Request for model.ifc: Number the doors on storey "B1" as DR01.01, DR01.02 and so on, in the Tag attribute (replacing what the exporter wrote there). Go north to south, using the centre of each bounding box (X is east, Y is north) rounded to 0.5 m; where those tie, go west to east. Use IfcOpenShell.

First a look at what the model holds.

```python
import ifcopenshell
import ifcopenshell.util.element
import ifcopenshell.util.placement

model = ifcopenshell.open("model.ifc")
print(model.schema)
storey = next(s for s in model.by_type("IfcBuildingStorey") if s.Name == "B1")
doors = [e for e in ifcopenshell.util.element.get_decomposition(storey) if e.is_a("IfcDoor")]
for e in sorted(doors, key=lambda e: e.id()):
    origin = ifcopenshell.util.placement.get_local_placement(e.ObjectPlacement)[:3, 3]
    print(e.id(), e.Tag, e.Name, origin.round(2) + 0.0, sep=" | ")
```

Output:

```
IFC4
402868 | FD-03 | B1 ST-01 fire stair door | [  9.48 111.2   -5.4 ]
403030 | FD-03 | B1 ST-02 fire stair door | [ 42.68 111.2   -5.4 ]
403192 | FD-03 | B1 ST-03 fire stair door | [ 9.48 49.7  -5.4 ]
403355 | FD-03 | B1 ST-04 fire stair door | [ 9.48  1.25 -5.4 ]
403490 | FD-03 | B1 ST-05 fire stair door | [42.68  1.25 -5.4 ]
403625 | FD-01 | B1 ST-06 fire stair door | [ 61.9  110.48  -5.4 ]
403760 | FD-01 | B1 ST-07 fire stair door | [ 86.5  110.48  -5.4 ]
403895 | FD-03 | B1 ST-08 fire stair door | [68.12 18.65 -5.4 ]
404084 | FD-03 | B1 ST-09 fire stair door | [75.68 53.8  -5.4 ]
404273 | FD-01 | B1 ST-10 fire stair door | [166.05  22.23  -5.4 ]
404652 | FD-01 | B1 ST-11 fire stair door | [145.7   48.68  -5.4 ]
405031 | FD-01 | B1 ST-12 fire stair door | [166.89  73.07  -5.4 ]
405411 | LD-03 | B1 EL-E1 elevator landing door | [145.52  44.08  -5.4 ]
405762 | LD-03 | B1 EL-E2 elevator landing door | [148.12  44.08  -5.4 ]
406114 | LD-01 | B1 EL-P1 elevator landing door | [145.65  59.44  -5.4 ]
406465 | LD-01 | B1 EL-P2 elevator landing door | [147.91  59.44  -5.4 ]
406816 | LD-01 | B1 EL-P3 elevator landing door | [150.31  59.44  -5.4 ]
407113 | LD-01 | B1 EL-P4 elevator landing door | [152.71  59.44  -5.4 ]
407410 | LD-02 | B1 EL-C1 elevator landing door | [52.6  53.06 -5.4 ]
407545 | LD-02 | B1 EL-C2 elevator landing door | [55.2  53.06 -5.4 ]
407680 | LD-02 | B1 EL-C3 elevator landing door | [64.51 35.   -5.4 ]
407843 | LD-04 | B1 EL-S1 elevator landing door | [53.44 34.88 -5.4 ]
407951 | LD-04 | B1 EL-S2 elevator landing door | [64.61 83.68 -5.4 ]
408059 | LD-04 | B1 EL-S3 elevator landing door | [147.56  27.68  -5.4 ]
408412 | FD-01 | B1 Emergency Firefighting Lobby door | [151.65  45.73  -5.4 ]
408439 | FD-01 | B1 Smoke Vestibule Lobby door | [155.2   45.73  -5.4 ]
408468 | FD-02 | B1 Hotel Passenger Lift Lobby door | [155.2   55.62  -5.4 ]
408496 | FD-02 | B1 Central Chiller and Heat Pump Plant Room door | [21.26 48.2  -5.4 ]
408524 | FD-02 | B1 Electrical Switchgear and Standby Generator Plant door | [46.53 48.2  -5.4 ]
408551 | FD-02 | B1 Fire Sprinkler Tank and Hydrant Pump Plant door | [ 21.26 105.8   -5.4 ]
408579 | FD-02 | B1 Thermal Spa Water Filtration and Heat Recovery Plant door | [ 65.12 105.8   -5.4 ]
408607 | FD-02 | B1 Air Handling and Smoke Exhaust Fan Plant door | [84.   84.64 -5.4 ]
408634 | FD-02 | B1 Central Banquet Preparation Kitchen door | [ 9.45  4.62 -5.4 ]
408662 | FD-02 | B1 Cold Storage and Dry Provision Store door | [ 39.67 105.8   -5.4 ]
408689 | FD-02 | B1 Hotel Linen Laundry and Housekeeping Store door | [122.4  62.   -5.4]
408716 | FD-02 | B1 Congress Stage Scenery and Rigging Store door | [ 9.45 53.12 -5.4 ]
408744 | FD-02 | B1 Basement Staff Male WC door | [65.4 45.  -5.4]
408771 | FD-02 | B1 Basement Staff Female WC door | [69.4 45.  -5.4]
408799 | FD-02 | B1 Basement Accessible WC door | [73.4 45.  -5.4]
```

```python
import ifcopenshell
import ifcopenshell.geom
import ifcopenshell.util.element
import ifcopenshell.util.shape

model = ifcopenshell.open("model.ifc")
settings = ifcopenshell.geom.settings()
settings.set("use-world-coords", True)


def centre(element):
    shape = ifcopenshell.geom.create_shape(settings, element)
    return ifcopenshell.util.shape.get_bbox_centroid(shape.geometry)


storey = next(s for s in model.by_type("IfcBuildingStorey") if s.Name == "B1")
doors = [e for e in ifcopenshell.util.element.get_decomposition(storey) if e.is_a("IfcDoor")]

# Insertion points can sit at a corner or the storey origin, so sort by the geometry (in metres).
centres = {e: centre(e) for e in doors}
doors.sort(key=lambda e: (-round(centres[e][1] / 0.5), centres[e][0]))

for i, e in enumerate(doors, start=1):
    number = f"DR01.{i:02d}"
    e.Tag = number
    print(e.id(), number)

model.write("model-out.ifc")
```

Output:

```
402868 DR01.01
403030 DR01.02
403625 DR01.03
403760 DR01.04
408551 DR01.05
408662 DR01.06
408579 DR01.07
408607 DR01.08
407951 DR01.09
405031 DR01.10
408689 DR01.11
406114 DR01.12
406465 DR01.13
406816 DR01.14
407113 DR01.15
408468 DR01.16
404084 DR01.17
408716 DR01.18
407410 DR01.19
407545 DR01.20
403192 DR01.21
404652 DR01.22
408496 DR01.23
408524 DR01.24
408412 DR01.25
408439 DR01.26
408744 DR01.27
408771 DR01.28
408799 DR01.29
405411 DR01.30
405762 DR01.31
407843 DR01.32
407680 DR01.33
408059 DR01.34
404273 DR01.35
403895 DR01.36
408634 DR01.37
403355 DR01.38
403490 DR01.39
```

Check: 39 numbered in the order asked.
